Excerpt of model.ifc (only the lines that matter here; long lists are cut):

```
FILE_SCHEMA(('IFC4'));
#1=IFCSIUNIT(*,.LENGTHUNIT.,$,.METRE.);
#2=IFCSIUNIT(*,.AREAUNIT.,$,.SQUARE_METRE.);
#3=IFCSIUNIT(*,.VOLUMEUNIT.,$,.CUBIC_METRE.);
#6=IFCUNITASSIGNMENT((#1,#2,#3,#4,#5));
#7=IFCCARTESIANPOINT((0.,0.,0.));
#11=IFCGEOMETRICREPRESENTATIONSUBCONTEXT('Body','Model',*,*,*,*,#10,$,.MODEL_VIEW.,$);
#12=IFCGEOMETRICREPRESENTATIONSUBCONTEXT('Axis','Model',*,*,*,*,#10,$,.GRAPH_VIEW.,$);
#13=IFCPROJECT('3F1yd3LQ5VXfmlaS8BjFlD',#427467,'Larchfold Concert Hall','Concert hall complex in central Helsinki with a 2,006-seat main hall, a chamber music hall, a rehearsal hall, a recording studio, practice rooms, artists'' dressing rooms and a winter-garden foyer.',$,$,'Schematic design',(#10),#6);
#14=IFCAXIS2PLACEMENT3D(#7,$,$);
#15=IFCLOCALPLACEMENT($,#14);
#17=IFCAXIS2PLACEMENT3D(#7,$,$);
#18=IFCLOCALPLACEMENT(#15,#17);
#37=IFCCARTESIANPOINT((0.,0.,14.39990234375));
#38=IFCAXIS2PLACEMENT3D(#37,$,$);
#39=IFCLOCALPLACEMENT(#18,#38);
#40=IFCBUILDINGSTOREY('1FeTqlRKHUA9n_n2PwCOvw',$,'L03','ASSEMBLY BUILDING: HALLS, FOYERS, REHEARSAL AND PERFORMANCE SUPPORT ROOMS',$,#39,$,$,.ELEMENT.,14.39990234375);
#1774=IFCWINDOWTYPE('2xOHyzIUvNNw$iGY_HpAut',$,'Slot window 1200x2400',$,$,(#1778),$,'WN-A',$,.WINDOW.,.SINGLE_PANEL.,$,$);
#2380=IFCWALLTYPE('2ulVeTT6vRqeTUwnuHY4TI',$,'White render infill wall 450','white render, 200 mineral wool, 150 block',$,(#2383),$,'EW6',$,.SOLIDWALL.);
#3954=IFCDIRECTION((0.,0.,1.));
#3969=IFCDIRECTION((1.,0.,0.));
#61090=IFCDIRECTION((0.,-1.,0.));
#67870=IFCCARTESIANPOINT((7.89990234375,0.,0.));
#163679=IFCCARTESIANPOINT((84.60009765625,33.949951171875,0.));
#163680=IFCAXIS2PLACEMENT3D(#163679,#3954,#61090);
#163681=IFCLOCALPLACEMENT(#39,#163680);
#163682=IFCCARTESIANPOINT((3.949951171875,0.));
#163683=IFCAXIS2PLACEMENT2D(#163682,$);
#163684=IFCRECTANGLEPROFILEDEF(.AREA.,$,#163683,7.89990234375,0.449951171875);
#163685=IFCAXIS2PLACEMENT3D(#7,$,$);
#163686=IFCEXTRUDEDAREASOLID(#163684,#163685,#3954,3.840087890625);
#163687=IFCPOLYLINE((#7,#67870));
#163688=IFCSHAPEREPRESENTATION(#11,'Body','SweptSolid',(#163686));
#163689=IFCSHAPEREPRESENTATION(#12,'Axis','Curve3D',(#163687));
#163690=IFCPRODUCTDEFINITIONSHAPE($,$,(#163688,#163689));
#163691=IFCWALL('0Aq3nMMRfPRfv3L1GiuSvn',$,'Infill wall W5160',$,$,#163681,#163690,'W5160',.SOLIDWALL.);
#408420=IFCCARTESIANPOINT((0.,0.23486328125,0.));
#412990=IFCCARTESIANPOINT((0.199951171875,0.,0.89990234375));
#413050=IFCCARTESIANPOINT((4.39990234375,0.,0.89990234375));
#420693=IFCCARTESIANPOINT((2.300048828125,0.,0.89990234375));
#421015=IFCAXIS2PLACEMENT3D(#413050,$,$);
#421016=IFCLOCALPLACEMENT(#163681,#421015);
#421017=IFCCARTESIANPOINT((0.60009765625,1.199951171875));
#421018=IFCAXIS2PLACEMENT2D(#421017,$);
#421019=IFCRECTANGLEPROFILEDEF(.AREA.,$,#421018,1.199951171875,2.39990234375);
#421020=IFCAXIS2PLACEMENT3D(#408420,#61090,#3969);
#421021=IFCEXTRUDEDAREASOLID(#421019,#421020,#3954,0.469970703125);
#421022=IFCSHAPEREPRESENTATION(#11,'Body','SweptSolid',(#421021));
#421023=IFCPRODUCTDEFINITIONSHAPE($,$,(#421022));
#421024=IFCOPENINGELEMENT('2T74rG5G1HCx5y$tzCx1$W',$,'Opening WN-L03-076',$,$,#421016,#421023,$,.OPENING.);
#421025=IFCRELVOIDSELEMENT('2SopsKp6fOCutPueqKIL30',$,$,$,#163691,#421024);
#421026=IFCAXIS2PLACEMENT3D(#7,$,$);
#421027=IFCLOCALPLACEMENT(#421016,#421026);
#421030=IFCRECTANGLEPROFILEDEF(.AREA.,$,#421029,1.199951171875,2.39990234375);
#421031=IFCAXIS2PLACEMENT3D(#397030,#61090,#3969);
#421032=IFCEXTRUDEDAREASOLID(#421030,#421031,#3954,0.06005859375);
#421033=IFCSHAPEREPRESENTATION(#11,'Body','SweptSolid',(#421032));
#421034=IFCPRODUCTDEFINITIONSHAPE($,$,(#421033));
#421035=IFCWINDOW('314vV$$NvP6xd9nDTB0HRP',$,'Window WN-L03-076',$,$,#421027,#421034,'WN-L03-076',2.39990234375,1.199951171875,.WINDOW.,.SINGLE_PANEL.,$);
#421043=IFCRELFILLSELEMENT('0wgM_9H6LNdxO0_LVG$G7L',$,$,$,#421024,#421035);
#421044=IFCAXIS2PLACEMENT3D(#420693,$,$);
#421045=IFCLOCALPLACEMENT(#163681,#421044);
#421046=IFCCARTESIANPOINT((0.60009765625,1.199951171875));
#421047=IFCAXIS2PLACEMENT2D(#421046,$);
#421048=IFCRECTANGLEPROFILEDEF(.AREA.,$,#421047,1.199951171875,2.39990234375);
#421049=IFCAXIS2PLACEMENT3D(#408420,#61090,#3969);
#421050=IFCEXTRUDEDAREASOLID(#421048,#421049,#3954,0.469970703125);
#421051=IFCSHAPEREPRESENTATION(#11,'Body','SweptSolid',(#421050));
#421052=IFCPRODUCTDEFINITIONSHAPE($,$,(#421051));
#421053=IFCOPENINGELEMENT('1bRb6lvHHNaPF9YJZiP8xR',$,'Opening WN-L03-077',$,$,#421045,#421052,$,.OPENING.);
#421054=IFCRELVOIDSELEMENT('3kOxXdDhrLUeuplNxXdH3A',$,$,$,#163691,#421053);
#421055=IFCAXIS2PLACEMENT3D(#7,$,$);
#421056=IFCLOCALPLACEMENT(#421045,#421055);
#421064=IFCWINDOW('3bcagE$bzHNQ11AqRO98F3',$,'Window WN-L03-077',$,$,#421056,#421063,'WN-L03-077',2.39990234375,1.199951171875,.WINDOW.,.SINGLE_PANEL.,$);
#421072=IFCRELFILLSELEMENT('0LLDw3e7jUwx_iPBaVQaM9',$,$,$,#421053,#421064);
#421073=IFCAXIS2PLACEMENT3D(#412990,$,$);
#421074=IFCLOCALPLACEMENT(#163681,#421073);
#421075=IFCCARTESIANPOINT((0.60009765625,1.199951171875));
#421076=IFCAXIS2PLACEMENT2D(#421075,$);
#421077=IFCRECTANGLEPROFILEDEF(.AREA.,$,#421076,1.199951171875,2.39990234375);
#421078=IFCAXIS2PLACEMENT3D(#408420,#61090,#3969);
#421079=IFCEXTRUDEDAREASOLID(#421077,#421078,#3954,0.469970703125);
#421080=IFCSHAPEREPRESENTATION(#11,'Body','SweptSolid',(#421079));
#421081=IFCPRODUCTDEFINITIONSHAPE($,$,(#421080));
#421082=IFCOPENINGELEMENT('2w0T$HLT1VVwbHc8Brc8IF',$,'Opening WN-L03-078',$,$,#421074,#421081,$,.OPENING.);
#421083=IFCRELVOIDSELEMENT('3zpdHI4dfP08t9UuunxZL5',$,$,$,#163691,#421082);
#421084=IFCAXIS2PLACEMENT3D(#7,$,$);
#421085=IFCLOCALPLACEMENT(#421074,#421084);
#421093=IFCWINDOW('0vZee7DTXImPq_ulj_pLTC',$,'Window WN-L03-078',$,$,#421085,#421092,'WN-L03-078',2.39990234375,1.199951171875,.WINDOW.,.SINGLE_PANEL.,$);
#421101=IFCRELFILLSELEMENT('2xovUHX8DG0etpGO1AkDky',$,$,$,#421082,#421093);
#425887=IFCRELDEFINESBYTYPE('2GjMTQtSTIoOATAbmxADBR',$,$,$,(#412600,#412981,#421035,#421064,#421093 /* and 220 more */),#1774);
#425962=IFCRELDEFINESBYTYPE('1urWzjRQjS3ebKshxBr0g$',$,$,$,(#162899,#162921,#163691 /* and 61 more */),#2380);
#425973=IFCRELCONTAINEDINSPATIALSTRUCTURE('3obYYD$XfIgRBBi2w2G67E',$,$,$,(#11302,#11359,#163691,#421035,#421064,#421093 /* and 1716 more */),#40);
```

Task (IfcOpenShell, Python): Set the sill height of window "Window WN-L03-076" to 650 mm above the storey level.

```python
import numpy as np
import ifcopenshell
import ifcopenshell.api.geometry
import ifcopenshell.geom
import ifcopenshell.util.element
import ifcopenshell.util.placement
import ifcopenshell.util.shape
import ifcopenshell.util.unit

model = ifcopenshell.open("model.ifc")
unit_scale = ifcopenshell.util.unit.calculate_unit_scale(model)

window = model.by_guid("314vV$$NvP6xd9nDTB0HRP")
opening = window.FillsVoids[0].RelatingOpeningElement
storey = ifcopenshell.util.element.get_container(window, ifc_class="IfcBuildingStorey")
level = ifcopenshell.util.placement.get_local_placement(storey.ObjectPlacement)[2, 3]

# The opening's origin need not be at the sill, so measure its lowest point.
shape = ifcopenshell.geom.create_shape(ifcopenshell.geom.settings(), opening)
bottom = ifcopenshell.util.shape.get_shape_bottom_elevation(shape, shape.geometry) / unit_scale
dz = level + 0.65 - bottom

shift = np.array([0.0, 0.0, dz])
# The window is placed relative to its opening, so it follows when the opening moves.
matrix = ifcopenshell.util.placement.get_local_placement(opening.ObjectPlacement)
matrix[:3, 3] += shift
ifcopenshell.api.geometry.edit_object_placement(
    model, product=opening, matrix=matrix, is_si=False, should_transform_children=True
)

print(f"moved by {dz * unit_scale:+.3f} m")

model.write("model_edited.ifc")
```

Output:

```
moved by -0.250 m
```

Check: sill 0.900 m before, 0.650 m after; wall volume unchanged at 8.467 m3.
